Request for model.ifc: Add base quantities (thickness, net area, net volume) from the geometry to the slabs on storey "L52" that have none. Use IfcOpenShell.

First a look at what the model holds.

```python
import ifcopenshell
import ifcopenshell.util.element
import ifcopenshell.util.unit

model = ifcopenshell.open("model.ifc")
print(model.schema)
for unit_type in ("LENGTHUNIT", "AREAUNIT", "VOLUMEUNIT"):
    print(unit_type, ifcopenshell.util.unit.calculate_unit_scale(model, unit_type))
storey = next(s for s in model.by_type("IfcBuildingStorey") if s.Name == "L52")
slabs = [e for e in ifcopenshell.util.element.get_decomposition(storey) if e.is_a("IfcSlab")]
for e in sorted(slabs, key=lambda e: e.id()):
    print(e.id(), e.is_a(), e.Name, list(ifcopenshell.util.element.get_psets(e, qtos_only=True)), sep=" | ")
```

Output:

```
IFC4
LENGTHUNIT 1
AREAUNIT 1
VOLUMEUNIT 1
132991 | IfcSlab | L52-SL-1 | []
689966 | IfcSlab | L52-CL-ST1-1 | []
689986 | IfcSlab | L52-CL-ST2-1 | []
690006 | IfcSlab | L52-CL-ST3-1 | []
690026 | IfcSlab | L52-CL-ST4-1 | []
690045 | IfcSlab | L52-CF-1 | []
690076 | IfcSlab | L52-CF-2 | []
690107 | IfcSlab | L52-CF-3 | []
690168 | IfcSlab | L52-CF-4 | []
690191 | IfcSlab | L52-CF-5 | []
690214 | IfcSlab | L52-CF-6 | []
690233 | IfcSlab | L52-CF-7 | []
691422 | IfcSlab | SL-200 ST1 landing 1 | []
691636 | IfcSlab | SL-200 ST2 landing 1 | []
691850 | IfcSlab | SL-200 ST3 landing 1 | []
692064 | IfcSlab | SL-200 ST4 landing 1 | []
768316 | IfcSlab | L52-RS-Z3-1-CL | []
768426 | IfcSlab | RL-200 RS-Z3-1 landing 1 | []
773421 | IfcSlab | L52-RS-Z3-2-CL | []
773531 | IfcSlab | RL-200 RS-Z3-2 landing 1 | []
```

```python
import ifcopenshell
import ifcopenshell.api.pset
import ifcopenshell.geom
import ifcopenshell.util.element
import ifcopenshell.util.shape
import ifcopenshell.util.unit

model = ifcopenshell.open("model.ifc")
unit_scale = ifcopenshell.util.unit.calculate_unit_scale(model)
area_scale = ifcopenshell.util.unit.calculate_unit_scale(model, "AREAUNIT")
volume_scale = ifcopenshell.util.unit.calculate_unit_scale(model, "VOLUMEUNIT")
settings = ifcopenshell.geom.settings()

storey = next(s for s in model.by_type("IfcBuildingStorey") if s.Name == "L52")
slabs = [e for e in ifcopenshell.util.element.get_decomposition(storey) if e.is_a("IfcSlab")]

for e in sorted(slabs, key=lambda e: e.id()):
    if ifcopenshell.util.element.get_psets(e, qtos_only=True, should_inherit=False):
        continue
    # Geometry comes back in metres, in the element's own axes.
    shape = ifcopenshell.geom.create_shape(settings, e)
    values = {
        "Width": ifcopenshell.util.shape.get_z(shape.geometry) / unit_scale,
        "NetArea": ifcopenshell.util.shape.get_footprint_area(shape.geometry) / area_scale,
        "NetVolume": ifcopenshell.util.shape.get_volume(shape.geometry) / volume_scale,
    }
    qto = ifcopenshell.api.pset.add_qto(model, product=e, name="Qto_SlabBaseQuantities")
    ifcopenshell.api.pset.edit_qto(model, qto=qto, properties=values)
    print(e.id(), {k: round(v, 3) for k, v in values.items()})

model.write("model_updated.ifc")
```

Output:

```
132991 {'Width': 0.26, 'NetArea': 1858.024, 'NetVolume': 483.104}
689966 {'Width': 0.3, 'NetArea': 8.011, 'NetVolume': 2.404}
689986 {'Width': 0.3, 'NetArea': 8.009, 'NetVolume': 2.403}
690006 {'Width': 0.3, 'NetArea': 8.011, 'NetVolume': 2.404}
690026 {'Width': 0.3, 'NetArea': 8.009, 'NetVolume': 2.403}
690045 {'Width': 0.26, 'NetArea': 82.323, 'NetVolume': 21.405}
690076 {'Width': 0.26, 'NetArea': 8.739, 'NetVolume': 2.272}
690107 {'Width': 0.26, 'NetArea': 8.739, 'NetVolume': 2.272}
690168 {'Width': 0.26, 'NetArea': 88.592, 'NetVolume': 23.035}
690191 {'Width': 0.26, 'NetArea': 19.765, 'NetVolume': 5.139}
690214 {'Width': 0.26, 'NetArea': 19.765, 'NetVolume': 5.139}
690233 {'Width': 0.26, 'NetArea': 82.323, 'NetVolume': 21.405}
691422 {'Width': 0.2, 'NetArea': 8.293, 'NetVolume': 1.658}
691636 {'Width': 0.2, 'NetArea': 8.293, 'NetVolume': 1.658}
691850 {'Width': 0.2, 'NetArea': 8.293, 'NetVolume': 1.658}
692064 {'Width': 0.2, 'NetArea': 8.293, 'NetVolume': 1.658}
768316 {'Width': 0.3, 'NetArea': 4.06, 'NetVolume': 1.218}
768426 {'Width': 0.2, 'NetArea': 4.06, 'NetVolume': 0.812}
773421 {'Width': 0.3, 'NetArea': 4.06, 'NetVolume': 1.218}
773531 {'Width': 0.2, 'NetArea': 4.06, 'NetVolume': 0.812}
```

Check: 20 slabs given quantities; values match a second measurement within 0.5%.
